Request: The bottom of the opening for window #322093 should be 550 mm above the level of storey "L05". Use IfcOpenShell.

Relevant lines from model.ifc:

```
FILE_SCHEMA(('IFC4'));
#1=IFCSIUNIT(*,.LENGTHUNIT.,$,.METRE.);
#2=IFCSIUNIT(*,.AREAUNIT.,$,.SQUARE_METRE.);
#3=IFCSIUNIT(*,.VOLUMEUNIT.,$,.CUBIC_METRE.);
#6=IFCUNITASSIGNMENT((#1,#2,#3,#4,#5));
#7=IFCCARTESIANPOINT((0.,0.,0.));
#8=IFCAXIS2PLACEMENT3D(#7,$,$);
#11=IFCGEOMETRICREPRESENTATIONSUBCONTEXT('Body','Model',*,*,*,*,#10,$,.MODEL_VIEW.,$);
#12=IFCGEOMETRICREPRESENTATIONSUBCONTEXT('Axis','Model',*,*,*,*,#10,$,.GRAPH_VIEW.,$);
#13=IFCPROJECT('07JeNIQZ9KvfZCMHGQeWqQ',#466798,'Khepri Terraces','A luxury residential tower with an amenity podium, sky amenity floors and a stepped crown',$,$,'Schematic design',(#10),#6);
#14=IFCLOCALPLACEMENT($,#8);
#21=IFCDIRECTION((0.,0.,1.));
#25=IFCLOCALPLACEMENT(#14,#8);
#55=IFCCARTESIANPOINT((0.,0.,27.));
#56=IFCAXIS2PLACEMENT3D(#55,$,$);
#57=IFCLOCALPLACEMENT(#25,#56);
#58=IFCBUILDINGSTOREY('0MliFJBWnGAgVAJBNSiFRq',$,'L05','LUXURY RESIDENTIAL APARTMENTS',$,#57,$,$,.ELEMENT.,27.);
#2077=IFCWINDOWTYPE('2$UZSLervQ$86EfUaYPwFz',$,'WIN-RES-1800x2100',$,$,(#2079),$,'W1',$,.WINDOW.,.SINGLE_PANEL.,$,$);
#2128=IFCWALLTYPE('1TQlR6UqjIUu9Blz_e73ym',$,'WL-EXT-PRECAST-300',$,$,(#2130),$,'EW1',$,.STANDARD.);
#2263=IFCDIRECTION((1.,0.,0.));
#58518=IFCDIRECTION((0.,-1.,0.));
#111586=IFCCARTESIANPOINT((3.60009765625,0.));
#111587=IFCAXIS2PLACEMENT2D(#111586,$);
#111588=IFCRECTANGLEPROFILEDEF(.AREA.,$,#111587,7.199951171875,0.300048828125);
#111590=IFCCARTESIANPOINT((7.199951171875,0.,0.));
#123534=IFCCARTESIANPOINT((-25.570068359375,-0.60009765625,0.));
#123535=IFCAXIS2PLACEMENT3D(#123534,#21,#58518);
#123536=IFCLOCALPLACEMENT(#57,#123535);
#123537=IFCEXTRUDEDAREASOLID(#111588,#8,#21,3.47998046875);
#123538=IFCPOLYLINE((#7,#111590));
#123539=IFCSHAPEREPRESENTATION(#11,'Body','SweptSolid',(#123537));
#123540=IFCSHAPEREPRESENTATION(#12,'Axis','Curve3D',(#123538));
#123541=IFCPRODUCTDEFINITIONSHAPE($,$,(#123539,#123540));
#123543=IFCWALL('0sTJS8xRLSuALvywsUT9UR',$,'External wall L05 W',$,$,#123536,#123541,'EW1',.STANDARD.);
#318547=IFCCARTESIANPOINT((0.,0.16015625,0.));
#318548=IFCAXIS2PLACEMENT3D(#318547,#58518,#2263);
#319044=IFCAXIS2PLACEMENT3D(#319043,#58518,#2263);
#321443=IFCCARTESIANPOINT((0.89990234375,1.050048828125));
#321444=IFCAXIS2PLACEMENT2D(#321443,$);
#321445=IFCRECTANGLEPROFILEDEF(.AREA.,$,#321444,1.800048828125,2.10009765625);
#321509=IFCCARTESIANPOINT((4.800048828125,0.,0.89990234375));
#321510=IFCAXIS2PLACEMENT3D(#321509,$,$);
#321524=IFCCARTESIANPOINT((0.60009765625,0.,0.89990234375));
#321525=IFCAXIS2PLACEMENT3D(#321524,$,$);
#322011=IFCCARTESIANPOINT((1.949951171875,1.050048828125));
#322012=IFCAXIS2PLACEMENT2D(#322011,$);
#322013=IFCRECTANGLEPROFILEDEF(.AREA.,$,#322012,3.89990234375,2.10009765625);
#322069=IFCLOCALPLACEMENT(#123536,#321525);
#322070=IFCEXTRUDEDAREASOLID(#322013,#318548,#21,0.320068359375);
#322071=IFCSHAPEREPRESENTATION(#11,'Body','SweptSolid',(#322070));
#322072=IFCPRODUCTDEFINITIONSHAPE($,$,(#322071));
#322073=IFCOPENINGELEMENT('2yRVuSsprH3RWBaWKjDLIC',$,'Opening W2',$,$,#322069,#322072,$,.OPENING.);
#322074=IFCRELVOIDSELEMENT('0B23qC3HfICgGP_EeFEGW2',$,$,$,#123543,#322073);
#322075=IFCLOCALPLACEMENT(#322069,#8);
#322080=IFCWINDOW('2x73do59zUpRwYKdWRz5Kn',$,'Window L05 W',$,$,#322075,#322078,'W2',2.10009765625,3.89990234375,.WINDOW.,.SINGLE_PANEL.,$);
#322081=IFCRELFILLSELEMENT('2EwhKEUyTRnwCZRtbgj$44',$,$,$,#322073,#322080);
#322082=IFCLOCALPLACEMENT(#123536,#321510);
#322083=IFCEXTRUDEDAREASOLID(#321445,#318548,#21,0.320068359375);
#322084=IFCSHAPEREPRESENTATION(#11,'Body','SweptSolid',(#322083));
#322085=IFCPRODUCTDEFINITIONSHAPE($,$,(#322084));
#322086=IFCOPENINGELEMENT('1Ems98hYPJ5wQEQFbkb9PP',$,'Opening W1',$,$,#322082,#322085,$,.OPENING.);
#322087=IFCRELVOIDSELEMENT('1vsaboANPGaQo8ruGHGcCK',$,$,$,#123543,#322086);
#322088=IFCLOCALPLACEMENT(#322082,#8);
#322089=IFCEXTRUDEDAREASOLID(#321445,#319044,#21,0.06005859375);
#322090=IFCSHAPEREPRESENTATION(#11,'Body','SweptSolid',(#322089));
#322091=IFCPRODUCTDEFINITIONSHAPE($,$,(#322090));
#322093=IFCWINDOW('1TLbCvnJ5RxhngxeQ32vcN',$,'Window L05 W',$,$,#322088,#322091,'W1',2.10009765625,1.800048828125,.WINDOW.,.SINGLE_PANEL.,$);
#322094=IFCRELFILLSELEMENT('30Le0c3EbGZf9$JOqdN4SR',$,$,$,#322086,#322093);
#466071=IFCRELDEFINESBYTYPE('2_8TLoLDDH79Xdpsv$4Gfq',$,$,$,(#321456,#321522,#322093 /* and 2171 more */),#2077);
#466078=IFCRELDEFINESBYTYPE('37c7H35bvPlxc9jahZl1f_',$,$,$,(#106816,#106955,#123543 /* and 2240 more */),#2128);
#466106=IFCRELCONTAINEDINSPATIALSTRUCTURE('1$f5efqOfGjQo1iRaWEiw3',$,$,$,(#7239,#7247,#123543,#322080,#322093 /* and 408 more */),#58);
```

```python
import numpy as np
import ifcopenshell
import ifcopenshell.api.geometry
import ifcopenshell.geom
import ifcopenshell.util.element
import ifcopenshell.util.placement
import ifcopenshell.util.shape
import ifcopenshell.util.unit

model = ifcopenshell.open("model.ifc")
unit_scale = ifcopenshell.util.unit.calculate_unit_scale(model)

window = model.by_guid("1TLbCvnJ5RxhngxeQ32vcN")
opening = window.FillsVoids[0].RelatingOpeningElement
storey = ifcopenshell.util.element.get_container(window, ifc_class="IfcBuildingStorey")
level = ifcopenshell.util.placement.get_local_placement(storey.ObjectPlacement)[2, 3]

# The opening's origin need not be at the sill, so measure its lowest point.
shape = ifcopenshell.geom.create_shape(ifcopenshell.geom.settings(), opening)
bottom = ifcopenshell.util.shape.get_shape_bottom_elevation(shape, shape.geometry) / unit_scale
dz = level + 0.55 - bottom

shift = np.array([0.0, 0.0, dz])
# The window is placed relative to its opening, so it follows when the opening moves.
matrix = ifcopenshell.util.placement.get_local_placement(opening.ObjectPlacement)
matrix[:3, 3] += shift
ifcopenshell.api.geometry.edit_object_placement(
    model, product=opening, matrix=matrix, is_si=False, should_transform_children=True
)

print(f"moved by {dz * unit_scale:+.3f} m")

model.write("model_updated.ifc")
```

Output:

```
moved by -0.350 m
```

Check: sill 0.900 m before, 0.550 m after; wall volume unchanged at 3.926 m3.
